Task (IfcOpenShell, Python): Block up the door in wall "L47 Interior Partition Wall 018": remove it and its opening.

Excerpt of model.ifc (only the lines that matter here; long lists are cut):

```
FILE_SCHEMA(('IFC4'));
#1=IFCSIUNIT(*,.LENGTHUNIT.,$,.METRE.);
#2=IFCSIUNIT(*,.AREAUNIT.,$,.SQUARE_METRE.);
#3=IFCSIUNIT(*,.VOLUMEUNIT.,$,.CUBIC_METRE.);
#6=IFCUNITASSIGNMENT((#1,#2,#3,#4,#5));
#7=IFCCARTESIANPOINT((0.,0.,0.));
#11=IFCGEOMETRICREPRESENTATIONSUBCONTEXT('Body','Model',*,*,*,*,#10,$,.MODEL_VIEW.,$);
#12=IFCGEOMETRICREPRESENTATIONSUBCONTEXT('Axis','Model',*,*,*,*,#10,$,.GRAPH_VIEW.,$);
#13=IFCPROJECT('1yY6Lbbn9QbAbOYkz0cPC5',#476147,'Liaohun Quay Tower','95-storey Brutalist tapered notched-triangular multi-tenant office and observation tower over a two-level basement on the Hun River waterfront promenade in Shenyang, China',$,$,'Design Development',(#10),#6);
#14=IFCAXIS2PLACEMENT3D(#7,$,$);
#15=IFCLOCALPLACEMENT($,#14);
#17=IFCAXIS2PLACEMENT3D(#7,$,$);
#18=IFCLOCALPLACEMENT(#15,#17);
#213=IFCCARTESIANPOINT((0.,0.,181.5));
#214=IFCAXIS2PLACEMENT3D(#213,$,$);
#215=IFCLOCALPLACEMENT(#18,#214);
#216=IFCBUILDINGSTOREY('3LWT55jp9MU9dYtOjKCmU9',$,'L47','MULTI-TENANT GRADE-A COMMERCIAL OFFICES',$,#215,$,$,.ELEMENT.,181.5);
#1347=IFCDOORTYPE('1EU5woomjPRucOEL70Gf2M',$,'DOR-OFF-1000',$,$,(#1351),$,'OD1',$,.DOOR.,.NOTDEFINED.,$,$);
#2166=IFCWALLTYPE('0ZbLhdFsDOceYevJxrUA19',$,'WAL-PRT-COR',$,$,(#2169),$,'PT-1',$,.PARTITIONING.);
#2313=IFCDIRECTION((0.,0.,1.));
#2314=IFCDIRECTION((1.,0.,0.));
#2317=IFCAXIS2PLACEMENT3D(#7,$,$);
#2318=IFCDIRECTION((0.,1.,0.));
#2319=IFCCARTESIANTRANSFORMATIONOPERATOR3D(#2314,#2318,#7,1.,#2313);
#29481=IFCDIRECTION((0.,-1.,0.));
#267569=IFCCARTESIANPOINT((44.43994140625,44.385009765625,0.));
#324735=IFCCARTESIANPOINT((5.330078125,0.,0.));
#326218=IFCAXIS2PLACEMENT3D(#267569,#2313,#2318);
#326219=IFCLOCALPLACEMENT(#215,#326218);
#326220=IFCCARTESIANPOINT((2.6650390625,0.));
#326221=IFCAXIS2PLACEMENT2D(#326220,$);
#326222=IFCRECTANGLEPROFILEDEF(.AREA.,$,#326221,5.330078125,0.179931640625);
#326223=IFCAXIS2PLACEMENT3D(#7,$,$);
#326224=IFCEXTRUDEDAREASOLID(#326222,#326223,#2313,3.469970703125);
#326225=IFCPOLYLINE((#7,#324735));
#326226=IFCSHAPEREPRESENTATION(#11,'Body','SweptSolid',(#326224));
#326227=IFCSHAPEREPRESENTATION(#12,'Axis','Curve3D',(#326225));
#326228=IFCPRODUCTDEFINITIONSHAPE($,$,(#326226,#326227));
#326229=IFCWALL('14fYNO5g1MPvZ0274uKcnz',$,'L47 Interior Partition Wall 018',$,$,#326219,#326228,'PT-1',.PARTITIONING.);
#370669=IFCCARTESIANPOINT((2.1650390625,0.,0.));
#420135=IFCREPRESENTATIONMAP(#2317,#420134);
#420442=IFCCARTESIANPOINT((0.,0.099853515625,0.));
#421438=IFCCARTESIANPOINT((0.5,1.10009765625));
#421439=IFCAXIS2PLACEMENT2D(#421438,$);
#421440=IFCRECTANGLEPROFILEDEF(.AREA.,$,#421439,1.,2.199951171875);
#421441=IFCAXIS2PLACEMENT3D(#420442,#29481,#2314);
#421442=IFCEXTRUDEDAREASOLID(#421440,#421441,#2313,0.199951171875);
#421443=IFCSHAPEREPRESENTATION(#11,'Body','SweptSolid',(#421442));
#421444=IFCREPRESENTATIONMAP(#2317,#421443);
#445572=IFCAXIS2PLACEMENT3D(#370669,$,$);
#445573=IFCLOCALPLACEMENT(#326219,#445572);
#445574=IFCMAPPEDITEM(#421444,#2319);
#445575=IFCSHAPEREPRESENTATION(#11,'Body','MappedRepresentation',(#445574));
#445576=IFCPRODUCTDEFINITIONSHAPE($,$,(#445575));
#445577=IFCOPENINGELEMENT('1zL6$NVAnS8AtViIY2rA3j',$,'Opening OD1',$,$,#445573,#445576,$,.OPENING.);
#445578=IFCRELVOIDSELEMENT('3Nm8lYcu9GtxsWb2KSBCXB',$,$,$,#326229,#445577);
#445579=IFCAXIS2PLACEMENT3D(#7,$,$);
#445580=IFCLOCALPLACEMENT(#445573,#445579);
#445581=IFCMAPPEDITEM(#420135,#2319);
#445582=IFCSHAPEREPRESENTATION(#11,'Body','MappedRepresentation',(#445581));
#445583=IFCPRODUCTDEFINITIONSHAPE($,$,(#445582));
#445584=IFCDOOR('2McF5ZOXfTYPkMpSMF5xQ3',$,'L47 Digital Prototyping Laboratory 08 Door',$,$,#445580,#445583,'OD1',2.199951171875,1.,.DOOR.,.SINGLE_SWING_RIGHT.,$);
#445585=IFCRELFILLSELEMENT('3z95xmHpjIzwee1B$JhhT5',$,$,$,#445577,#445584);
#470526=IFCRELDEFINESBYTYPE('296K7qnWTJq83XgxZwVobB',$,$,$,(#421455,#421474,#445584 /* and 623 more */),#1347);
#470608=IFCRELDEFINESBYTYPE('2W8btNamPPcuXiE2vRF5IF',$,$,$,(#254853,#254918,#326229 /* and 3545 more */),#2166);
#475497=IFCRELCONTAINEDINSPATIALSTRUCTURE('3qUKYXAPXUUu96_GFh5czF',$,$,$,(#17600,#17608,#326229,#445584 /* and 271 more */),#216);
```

```python
import ifcopenshell
import ifcopenshell.api.feature
import ifcopenshell.api.root
import ifcopenshell.geom
import ifcopenshell.util.shape

model = ifcopenshell.open("model.ifc")
settings = ifcopenshell.geom.settings()


def volume(element):
    """Net volume in cubic metres, openings subtracted."""
    shape = ifcopenshell.geom.create_shape(settings, element)
    return ifcopenshell.util.shape.get_volume(shape.geometry)


door = model.by_id(445584)
opening = door.FillsVoids[0].RelatingOpeningElement
wall = opening.VoidsElements[0].RelatingBuildingElement
before = volume(wall)

ifcopenshell.api.root.remove_product(model, product=door)
ifcopenshell.api.feature.remove_feature(model, feature=opening)

after = volume(wall)

print(f"wall volume {before:.3f} -> {after:.3f} m3")

model.write("model_v2.ifc")
```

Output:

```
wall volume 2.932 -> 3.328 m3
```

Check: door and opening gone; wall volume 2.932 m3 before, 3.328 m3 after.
